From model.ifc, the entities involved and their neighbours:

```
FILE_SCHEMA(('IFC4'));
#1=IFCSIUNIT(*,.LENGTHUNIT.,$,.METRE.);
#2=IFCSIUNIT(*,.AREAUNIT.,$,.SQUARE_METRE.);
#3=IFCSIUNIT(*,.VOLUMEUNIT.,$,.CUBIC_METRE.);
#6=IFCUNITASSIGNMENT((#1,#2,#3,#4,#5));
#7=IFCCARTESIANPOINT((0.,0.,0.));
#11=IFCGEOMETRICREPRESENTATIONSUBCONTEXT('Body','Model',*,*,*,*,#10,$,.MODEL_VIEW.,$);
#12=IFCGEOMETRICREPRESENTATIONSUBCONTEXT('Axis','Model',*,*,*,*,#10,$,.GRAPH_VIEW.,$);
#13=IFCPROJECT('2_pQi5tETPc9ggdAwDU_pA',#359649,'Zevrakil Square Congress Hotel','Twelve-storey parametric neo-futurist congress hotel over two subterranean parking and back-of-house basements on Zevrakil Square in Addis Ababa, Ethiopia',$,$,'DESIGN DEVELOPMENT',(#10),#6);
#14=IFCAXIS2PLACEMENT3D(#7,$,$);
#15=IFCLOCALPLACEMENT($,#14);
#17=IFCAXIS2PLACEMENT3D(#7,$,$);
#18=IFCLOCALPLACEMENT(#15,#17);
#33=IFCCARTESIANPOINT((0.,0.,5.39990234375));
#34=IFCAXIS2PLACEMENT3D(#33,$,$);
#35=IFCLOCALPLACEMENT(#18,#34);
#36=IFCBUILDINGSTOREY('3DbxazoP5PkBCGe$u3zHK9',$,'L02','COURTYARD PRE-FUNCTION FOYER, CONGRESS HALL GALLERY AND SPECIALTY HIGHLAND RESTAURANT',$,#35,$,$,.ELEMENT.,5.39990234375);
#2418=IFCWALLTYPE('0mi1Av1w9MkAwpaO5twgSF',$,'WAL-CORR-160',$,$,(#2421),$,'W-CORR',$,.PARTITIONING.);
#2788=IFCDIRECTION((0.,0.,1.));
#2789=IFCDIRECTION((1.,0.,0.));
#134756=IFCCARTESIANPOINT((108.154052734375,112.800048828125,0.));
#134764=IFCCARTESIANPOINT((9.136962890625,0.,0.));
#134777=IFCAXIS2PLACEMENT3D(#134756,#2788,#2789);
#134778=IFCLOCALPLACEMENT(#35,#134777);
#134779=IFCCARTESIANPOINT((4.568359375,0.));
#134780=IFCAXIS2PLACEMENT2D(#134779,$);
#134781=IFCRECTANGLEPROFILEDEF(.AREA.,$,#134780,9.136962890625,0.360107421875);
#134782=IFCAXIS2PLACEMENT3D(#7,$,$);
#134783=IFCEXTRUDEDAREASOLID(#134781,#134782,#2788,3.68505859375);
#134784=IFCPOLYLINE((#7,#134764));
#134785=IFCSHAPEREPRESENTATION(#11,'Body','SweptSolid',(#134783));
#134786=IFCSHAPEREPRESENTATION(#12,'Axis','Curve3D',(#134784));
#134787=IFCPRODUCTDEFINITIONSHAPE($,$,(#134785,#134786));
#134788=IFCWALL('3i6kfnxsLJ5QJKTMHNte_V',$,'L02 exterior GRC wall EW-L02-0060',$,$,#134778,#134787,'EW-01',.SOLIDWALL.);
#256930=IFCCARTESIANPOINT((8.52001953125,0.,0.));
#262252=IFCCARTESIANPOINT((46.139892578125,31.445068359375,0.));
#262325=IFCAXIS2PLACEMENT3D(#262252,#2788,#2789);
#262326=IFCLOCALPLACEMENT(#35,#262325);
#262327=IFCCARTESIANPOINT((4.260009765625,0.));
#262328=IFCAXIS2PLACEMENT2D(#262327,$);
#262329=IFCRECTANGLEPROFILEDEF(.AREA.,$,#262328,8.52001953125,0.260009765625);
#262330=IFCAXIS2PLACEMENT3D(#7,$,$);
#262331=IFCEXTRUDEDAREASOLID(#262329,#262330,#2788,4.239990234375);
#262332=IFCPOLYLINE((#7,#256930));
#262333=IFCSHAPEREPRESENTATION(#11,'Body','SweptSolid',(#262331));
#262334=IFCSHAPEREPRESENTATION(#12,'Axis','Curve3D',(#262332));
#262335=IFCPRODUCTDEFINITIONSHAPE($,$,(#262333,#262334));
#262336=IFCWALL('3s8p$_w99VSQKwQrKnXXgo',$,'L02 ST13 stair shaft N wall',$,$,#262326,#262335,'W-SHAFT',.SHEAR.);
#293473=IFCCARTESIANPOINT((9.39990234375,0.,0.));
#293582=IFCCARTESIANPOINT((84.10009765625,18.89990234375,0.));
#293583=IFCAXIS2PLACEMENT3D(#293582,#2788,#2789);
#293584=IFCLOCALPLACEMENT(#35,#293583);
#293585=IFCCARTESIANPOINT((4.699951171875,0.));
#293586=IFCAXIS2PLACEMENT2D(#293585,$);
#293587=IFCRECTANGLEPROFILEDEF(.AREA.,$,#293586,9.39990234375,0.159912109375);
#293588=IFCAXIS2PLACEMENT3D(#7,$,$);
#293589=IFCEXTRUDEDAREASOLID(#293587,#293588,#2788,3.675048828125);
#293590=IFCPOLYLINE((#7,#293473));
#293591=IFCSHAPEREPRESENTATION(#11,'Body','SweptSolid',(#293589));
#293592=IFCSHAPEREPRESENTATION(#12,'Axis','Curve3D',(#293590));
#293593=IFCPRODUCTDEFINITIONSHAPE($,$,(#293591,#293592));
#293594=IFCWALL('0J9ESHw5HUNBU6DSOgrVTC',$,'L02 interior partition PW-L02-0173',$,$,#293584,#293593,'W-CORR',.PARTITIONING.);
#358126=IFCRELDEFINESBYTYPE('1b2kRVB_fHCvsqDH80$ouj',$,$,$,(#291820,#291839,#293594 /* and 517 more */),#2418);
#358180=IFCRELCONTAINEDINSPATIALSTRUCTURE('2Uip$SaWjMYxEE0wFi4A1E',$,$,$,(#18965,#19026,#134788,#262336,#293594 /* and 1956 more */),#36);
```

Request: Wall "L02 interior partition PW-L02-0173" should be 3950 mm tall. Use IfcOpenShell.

```python
import ifcopenshell
import ifcopenshell.geom
import ifcopenshell.util.representation
import ifcopenshell.util.shape

model = ifcopenshell.open("model.ifc")
settings = ifcopenshell.geom.settings()


def volume(element):
    """Net volume in cubic metres, openings subtracted."""
    shape = ifcopenshell.geom.create_shape(settings, element)
    return ifcopenshell.util.shape.get_volume(shape.geometry)


wall = model.by_id(293594)
before = volume(wall)

body = ifcopenshell.util.representation.get_representation(wall, "Model", "Body")
solid = body.Items[0]
old_height = solid.Depth
solid.Depth = 3.95
after = volume(wall)

print(f"height {old_height:g} -> {solid.Depth:g}, volume {before:.3f} -> {after:.3f} m3")

model.write("model-out.ifc")
```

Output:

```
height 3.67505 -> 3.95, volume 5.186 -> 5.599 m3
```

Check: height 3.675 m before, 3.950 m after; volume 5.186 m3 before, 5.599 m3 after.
